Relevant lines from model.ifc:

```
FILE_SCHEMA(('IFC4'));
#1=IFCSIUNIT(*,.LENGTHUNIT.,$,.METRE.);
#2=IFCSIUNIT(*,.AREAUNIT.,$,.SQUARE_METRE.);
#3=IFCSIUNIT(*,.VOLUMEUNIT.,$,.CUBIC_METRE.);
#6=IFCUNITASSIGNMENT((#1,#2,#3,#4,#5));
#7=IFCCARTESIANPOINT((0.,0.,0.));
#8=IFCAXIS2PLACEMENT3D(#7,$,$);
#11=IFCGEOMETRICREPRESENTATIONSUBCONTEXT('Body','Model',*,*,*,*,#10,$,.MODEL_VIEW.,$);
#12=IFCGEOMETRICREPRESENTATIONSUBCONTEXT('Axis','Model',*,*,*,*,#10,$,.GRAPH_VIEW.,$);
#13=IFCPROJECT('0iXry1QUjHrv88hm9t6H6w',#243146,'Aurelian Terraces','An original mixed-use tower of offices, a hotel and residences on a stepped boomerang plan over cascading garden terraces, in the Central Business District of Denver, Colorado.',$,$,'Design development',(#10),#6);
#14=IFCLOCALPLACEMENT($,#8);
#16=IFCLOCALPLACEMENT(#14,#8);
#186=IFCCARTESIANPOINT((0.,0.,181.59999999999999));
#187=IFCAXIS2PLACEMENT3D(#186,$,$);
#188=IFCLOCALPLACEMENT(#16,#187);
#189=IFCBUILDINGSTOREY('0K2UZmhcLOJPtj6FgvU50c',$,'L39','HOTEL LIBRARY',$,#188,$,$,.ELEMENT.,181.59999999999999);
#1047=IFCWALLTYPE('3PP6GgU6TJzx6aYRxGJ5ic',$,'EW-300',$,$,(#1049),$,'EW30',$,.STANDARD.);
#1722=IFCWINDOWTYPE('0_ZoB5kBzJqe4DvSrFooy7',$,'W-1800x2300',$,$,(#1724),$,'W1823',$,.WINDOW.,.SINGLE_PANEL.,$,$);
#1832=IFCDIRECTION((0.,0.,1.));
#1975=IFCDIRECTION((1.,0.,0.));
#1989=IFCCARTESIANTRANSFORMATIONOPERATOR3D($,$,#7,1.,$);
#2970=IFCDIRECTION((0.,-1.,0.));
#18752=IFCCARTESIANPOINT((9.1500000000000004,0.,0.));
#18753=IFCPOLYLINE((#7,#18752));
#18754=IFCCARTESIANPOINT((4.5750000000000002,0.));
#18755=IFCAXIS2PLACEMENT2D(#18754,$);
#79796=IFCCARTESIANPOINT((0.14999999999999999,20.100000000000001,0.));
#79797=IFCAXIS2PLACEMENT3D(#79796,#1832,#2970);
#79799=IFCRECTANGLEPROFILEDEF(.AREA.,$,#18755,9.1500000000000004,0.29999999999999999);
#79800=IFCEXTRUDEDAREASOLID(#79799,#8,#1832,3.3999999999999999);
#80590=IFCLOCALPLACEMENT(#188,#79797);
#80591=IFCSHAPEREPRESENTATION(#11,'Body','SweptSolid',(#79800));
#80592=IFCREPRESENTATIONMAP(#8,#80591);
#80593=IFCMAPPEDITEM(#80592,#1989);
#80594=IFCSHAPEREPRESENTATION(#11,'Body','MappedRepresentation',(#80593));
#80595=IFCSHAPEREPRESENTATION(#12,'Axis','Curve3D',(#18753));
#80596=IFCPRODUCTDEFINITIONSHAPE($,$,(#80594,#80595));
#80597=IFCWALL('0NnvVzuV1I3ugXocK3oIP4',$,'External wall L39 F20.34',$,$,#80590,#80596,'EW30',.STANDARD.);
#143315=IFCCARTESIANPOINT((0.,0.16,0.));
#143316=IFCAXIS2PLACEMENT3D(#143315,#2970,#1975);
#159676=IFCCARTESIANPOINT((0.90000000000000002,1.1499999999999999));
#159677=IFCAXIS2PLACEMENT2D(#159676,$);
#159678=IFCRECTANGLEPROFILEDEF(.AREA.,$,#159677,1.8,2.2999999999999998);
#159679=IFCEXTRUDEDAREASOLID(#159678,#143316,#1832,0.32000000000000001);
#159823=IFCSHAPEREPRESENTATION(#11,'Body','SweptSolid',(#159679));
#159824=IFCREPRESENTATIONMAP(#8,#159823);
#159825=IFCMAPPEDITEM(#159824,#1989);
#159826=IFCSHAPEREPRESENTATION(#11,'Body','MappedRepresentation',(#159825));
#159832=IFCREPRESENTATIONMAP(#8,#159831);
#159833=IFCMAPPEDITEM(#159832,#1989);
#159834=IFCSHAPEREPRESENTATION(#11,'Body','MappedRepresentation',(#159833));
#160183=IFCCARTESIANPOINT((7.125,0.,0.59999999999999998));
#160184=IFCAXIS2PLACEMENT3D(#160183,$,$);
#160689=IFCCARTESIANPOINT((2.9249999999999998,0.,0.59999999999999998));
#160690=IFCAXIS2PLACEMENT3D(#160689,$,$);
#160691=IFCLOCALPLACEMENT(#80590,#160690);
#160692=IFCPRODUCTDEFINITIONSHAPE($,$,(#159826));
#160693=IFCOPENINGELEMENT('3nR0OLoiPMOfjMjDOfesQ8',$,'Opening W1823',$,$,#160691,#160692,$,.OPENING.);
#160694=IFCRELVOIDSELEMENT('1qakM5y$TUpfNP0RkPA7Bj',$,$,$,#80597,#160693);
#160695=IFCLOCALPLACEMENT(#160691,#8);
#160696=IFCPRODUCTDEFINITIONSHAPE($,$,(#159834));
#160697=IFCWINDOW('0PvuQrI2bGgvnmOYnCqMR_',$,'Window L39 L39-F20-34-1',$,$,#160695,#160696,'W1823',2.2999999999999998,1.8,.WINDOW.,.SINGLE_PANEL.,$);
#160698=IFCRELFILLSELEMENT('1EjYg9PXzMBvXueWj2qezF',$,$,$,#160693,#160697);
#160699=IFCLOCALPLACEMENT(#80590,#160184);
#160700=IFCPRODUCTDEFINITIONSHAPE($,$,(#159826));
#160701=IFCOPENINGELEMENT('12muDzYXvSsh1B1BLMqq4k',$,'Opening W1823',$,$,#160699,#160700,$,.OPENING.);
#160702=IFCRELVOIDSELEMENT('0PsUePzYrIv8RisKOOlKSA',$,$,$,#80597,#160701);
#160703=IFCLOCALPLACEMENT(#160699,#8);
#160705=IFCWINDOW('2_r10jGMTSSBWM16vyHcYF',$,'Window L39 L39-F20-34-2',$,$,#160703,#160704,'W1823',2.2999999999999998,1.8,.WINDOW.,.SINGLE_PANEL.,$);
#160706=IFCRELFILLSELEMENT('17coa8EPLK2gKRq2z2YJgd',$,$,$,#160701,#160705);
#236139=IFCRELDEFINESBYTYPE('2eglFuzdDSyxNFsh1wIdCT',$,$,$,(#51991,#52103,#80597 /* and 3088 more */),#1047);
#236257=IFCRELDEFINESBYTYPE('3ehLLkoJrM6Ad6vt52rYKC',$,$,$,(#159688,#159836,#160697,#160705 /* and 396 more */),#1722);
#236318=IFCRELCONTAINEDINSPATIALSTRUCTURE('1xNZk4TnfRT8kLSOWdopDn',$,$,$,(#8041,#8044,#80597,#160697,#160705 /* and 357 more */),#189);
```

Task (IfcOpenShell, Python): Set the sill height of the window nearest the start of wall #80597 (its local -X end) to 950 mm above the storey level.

```python
import numpy as np
import ifcopenshell
import ifcopenshell.api.geometry
import ifcopenshell.geom
import ifcopenshell.util.element
import ifcopenshell.util.placement
import ifcopenshell.util.shape
import ifcopenshell.util.unit

model = ifcopenshell.open("model.ifc")
unit_scale = ifcopenshell.util.unit.calculate_unit_scale(model)

window = model.by_id(160697)
opening = window.FillsVoids[0].RelatingOpeningElement
storey = ifcopenshell.util.element.get_container(window, ifc_class="IfcBuildingStorey")
level = ifcopenshell.util.placement.get_local_placement(storey.ObjectPlacement)[2, 3]

# The opening's origin need not be at the sill, so measure its lowest point.
shape = ifcopenshell.geom.create_shape(ifcopenshell.geom.settings(), opening)
bottom = ifcopenshell.util.shape.get_shape_bottom_elevation(shape, shape.geometry) / unit_scale
dz = level + 0.95 / unit_scale - bottom

shift = np.array([0.0, 0.0, dz])
# The window is placed relative to its opening, so it follows when the opening moves.
matrix = ifcopenshell.util.placement.get_local_placement(opening.ObjectPlacement)
matrix[:3, 3] += shift
ifcopenshell.api.geometry.edit_object_placement(
    model, product=opening, matrix=matrix, is_si=False, should_transform_children=True
)

print(f"moved by {dz * unit_scale:+.3f} m")

model.write("model_updated.ifc")
```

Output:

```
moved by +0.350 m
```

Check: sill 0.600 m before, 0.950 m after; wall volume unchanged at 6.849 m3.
